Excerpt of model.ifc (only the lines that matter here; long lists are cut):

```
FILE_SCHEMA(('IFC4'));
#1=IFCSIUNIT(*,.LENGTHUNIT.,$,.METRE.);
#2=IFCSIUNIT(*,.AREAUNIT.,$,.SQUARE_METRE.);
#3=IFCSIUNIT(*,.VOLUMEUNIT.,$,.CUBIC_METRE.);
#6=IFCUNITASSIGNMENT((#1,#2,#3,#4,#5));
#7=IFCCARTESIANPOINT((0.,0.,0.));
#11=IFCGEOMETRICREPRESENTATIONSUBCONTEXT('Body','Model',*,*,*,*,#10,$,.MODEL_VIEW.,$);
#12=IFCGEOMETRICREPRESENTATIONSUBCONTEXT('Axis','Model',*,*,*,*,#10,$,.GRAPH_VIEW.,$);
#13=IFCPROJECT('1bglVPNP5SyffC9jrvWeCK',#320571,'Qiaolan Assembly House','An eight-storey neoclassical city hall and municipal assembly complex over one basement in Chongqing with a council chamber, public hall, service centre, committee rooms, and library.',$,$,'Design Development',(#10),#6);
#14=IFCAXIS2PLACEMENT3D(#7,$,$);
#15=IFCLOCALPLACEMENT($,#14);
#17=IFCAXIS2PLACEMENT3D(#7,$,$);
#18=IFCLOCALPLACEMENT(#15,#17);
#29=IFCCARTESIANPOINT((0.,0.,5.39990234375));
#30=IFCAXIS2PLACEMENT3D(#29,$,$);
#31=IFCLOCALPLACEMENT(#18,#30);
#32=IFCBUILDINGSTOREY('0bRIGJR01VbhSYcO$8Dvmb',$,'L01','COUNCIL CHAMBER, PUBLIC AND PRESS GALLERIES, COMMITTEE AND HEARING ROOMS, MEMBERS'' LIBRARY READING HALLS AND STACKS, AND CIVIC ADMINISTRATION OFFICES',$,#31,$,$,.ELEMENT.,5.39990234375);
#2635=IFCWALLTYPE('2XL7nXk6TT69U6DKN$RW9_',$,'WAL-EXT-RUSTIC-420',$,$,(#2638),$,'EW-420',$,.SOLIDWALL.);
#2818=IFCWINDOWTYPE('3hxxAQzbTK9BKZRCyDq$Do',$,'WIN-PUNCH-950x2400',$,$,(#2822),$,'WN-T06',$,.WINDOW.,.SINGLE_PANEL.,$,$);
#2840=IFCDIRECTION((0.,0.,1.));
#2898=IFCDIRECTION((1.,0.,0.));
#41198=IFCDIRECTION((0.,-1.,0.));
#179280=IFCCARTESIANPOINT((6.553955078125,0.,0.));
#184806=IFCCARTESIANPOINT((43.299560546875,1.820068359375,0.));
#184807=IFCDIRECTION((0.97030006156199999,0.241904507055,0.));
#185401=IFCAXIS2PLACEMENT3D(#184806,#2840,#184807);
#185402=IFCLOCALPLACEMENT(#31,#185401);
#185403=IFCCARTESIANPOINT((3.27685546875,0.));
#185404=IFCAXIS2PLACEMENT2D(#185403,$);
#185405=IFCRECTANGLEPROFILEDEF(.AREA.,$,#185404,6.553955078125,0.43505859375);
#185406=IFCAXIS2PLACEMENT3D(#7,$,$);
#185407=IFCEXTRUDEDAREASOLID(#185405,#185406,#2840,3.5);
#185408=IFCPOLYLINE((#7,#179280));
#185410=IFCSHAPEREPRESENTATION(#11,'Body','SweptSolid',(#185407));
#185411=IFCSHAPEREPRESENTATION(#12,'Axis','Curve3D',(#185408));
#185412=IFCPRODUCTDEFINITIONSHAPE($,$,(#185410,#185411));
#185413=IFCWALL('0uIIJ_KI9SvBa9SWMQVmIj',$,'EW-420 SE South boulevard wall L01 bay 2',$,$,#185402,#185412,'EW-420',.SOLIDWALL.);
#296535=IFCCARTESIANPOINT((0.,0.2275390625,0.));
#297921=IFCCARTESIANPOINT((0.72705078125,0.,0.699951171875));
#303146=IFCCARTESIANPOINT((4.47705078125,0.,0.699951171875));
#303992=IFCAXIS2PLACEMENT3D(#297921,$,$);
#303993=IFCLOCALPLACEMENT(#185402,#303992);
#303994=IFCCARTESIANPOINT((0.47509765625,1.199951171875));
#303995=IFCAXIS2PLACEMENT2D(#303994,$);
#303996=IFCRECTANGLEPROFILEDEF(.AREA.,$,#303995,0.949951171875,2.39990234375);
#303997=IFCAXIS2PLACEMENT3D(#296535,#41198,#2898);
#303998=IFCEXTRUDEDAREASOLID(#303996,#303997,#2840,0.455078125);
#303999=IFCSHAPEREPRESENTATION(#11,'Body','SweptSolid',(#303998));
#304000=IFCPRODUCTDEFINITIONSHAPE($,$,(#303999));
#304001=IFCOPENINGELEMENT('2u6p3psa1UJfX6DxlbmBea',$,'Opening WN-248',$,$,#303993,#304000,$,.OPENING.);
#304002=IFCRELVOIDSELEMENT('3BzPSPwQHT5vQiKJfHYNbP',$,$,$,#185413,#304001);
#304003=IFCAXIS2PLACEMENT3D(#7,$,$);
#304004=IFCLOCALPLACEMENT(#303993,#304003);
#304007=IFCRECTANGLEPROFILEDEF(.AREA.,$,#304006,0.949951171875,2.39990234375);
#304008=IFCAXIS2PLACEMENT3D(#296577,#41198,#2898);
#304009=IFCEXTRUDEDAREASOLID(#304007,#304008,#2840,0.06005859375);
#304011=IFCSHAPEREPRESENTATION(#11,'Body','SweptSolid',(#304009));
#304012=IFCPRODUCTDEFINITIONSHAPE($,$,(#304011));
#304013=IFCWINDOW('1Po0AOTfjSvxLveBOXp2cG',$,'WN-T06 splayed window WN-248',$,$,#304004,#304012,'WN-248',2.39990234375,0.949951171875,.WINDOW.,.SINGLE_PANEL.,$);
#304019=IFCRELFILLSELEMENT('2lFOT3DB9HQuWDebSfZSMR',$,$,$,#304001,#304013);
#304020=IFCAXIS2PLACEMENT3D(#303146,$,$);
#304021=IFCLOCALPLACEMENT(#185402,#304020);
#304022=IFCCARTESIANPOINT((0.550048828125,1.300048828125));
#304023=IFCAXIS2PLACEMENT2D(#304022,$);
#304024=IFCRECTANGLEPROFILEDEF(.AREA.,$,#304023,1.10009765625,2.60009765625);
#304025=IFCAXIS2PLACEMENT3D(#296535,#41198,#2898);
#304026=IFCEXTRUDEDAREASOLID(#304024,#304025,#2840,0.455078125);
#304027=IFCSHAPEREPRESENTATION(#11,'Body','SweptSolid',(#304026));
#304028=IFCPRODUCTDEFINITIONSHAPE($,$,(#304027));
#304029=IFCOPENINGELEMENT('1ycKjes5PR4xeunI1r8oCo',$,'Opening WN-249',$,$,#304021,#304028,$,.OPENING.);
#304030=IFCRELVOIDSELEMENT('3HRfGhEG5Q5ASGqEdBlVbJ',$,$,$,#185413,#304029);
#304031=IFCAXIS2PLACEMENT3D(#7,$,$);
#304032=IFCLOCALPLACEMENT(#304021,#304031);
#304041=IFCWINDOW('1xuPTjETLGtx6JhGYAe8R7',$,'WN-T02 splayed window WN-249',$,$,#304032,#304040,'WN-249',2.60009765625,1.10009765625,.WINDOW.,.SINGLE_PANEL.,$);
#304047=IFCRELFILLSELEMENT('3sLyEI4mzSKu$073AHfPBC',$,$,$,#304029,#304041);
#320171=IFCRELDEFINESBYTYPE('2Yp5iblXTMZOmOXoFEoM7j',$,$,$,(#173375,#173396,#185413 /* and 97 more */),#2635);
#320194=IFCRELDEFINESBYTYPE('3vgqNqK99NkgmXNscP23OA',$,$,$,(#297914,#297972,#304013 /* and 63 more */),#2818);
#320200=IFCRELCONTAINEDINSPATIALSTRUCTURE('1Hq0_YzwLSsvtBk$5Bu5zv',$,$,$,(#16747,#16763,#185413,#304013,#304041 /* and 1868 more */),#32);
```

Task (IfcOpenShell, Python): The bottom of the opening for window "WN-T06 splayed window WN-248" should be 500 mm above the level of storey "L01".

```python
import numpy as np
import ifcopenshell
import ifcopenshell.api.geometry
import ifcopenshell.geom
import ifcopenshell.util.element
import ifcopenshell.util.placement
import ifcopenshell.util.shape
import ifcopenshell.util.unit

model = ifcopenshell.open("model.ifc")
unit_scale = ifcopenshell.util.unit.calculate_unit_scale(model)

window = model.by_id(304013)
opening = window.FillsVoids[0].RelatingOpeningElement
storey = ifcopenshell.util.element.get_container(window, ifc_class="IfcBuildingStorey")
level = ifcopenshell.util.placement.get_local_placement(storey.ObjectPlacement)[2, 3]

# The opening's origin need not be at the sill, so measure its lowest point.
shape = ifcopenshell.geom.create_shape(ifcopenshell.geom.settings(), opening)
bottom = ifcopenshell.util.shape.get_shape_bottom_elevation(shape, shape.geometry) / unit_scale
dz = level + 0.5 / unit_scale - bottom

shift = np.array([0.0, 0.0, dz])
# The window is placed relative to its opening, so it follows when the opening moves.
matrix = ifcopenshell.util.placement.get_local_placement(opening.ObjectPlacement)
matrix[:3, 3] += shift
ifcopenshell.api.geometry.edit_object_placement(
    model, product=opening, matrix=matrix, is_si=False, should_transform_children=True
)

print(f"moved by {dz * unit_scale:+.3f} m")

model.write("model_v2.ifc")
```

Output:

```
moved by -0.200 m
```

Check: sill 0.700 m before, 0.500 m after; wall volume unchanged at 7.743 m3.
